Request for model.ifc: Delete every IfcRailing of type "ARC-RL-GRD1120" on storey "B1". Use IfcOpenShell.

First a look at what the model holds.

```python
import ifcopenshell
import ifcopenshell.util.element

model = ifcopenshell.open("model.ifc")
print(model.schema)
storey = next(s for s in model.by_type("IfcBuildingStorey") if s.Name == "B1")
railings = [e for e in ifcopenshell.util.element.get_decomposition(storey) if e.is_a("IfcRailing")]
seen = {}
for e in railings:
    element_type = ifcopenshell.util.element.get_type(e)
    name = element_type.Name if element_type not in (None, e) else None
    seen[name] = seen.get(name, 0) + 1
for name, count in sorted(seen.items(), key=str):
    print(count, "x", name)
```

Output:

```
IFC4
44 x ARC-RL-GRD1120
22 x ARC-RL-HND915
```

```python
import ifcopenshell
import ifcopenshell.api.root
import ifcopenshell.util.element

model = ifcopenshell.open("model.ifc")

storey = next(s for s in model.by_type("IfcBuildingStorey") if s.Name == "B1")
railings = [e for e in ifcopenshell.util.element.get_decomposition(storey) if e.is_a("IfcRailing")]
targets = [e for e in railings if (t := ifcopenshell.util.element.get_type(e)) not in (None, e) and t.Name == "ARC-RL-GRD1120"]

for e in targets:
    ifcopenshell.api.root.remove_product(model, product=e)
print(len(targets), "removed")

model.write("model_v2.ifc")
```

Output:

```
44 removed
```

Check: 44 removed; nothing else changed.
